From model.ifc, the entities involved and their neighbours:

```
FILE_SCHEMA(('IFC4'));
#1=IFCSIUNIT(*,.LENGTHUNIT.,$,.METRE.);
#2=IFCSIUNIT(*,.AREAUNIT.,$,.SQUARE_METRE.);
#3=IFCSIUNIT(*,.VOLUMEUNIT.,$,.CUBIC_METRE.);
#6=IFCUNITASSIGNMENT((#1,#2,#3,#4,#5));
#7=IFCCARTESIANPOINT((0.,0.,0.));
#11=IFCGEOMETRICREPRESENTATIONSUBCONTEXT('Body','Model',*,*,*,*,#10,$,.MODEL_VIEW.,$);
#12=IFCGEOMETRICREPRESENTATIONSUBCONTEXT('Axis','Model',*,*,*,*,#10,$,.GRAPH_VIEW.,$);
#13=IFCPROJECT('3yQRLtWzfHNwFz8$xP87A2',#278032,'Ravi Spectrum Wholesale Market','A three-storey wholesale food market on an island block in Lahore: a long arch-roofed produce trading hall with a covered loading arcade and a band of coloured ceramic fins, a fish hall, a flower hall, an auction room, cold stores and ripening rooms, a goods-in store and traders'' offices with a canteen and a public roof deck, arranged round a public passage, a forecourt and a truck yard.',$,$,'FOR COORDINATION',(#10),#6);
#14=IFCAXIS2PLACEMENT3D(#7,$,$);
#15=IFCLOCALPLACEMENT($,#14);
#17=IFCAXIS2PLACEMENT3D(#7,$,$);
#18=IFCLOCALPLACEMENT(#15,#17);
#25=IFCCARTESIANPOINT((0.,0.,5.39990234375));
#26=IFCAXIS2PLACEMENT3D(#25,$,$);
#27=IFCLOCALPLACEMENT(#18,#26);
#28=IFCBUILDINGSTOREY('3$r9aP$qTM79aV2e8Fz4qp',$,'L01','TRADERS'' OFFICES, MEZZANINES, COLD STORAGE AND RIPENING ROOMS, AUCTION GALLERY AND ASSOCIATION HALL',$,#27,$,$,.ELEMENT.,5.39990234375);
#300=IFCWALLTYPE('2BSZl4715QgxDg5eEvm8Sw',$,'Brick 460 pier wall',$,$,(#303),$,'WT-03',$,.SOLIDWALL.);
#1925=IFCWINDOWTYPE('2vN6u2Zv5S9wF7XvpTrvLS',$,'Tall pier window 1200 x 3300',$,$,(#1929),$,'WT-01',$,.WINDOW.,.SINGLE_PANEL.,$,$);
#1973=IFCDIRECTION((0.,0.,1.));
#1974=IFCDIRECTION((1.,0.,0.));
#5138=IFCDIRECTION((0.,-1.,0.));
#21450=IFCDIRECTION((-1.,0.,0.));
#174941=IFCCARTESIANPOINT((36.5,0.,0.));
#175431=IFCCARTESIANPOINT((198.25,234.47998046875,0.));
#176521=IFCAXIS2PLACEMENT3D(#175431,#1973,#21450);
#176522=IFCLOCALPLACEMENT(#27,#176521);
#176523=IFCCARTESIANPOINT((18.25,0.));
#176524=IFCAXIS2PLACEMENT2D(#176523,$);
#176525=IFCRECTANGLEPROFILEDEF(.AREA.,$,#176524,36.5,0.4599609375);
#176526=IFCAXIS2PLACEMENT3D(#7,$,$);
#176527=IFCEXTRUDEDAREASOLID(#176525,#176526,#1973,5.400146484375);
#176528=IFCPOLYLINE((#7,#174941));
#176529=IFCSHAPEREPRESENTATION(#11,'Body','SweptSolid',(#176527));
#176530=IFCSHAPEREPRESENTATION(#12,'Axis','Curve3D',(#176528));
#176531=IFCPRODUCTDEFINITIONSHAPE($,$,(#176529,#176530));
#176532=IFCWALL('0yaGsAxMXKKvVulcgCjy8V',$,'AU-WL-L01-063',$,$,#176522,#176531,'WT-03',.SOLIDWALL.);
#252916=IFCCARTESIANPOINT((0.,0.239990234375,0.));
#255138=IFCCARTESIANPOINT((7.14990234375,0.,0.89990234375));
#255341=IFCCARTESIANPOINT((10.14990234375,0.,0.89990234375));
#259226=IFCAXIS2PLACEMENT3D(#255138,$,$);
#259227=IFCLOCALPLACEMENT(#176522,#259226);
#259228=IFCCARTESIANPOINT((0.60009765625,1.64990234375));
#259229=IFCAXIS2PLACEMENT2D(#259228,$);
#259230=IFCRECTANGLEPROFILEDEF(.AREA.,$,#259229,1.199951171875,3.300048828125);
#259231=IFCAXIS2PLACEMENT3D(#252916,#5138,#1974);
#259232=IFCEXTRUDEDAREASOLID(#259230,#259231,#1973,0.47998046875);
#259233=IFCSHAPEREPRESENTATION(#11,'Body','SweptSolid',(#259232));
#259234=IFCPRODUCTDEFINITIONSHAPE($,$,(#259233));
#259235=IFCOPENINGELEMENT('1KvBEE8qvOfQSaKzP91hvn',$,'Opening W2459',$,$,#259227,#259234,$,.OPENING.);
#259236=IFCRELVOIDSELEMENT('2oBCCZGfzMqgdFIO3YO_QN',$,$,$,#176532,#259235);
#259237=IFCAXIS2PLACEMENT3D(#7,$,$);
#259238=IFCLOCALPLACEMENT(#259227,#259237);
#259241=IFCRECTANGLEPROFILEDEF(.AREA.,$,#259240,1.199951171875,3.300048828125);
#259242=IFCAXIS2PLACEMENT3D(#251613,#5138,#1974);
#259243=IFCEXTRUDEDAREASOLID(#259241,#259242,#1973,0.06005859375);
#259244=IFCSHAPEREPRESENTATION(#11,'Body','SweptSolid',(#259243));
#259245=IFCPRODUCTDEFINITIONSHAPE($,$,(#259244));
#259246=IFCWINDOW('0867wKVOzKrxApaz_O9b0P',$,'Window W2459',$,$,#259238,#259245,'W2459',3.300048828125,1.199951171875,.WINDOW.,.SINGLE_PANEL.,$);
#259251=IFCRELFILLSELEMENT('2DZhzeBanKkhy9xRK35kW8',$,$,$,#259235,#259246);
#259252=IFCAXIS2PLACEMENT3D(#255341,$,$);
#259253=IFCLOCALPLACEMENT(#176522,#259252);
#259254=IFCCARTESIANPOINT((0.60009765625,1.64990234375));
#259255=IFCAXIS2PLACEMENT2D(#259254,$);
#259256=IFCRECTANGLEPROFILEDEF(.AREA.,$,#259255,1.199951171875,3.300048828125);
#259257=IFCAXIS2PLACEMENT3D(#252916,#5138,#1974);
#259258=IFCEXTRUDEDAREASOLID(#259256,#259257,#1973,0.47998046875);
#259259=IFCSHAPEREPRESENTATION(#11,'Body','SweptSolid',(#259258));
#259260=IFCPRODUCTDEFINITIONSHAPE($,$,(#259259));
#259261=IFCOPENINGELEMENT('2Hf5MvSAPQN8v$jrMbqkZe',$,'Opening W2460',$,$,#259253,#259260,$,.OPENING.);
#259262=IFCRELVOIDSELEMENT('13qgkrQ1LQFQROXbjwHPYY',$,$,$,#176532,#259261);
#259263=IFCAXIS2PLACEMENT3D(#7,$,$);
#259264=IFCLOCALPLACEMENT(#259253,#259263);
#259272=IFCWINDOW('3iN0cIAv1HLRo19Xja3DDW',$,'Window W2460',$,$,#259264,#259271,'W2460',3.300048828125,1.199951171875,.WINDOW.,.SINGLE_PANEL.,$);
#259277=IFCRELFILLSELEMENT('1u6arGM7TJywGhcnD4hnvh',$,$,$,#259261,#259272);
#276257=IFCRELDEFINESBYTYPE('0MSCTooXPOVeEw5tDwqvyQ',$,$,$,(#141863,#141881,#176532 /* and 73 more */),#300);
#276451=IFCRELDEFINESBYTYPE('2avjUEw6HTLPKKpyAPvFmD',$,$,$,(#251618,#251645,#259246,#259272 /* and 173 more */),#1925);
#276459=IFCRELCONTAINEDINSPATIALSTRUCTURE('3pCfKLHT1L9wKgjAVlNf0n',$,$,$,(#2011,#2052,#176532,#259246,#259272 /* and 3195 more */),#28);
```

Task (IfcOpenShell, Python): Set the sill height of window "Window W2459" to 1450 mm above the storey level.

```python
import numpy as np
import ifcopenshell
import ifcopenshell.api.geometry
import ifcopenshell.geom
import ifcopenshell.util.element
import ifcopenshell.util.placement
import ifcopenshell.util.shape
import ifcopenshell.util.unit

model = ifcopenshell.open("model.ifc")
unit_scale = ifcopenshell.util.unit.calculate_unit_scale(model)

window = model.by_guid("0867wKVOzKrxApaz_O9b0P")
opening = window.FillsVoids[0].RelatingOpeningElement
storey = ifcopenshell.util.element.get_container(window, ifc_class="IfcBuildingStorey")
level = ifcopenshell.util.placement.get_local_placement(storey.ObjectPlacement)[2, 3]

# The opening's origin need not be at the sill, so measure its lowest point.
shape = ifcopenshell.geom.create_shape(ifcopenshell.geom.settings(), opening)
bottom = ifcopenshell.util.shape.get_shape_bottom_elevation(shape, shape.geometry) / unit_scale
dz = level + 1.45 / unit_scale - bottom

shift = np.array([0.0, 0.0, dz])
# The window is placed relative to its opening, so it follows when the opening moves.
matrix = ifcopenshell.util.placement.get_local_placement(opening.ObjectPlacement)
matrix[:3, 3] += shift
ifcopenshell.api.geometry.edit_object_placement(
    model, product=opening, matrix=matrix, is_si=False, should_transform_children=True
)

print(f"moved by {dz * unit_scale:+.3f} m")

model.write("model_rev.ifc")
```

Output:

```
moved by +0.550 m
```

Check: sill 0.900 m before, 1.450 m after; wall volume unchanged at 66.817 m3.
